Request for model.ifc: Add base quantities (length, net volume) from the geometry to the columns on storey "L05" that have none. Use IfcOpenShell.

First a look at what the model holds.

```python
import ifcopenshell
import ifcopenshell.util.element
import ifcopenshell.util.unit

model = ifcopenshell.open("model.ifc")
print(model.schema)
for unit_type in ("LENGTHUNIT", "AREAUNIT", "VOLUMEUNIT"):
    print(unit_type, ifcopenshell.util.unit.calculate_unit_scale(model, unit_type))
storey = next(s for s in model.by_type("IfcBuildingStorey") if s.Name == "L05")
columns = [e for e in ifcopenshell.util.element.get_decomposition(storey) if e.is_a("IfcColumn")]
for e in sorted(columns, key=lambda e: e.id()):
    print(e.id(), e.is_a(), e.Name, list(ifcopenshell.util.element.get_psets(e, qtos_only=True)), sep=" | ")
```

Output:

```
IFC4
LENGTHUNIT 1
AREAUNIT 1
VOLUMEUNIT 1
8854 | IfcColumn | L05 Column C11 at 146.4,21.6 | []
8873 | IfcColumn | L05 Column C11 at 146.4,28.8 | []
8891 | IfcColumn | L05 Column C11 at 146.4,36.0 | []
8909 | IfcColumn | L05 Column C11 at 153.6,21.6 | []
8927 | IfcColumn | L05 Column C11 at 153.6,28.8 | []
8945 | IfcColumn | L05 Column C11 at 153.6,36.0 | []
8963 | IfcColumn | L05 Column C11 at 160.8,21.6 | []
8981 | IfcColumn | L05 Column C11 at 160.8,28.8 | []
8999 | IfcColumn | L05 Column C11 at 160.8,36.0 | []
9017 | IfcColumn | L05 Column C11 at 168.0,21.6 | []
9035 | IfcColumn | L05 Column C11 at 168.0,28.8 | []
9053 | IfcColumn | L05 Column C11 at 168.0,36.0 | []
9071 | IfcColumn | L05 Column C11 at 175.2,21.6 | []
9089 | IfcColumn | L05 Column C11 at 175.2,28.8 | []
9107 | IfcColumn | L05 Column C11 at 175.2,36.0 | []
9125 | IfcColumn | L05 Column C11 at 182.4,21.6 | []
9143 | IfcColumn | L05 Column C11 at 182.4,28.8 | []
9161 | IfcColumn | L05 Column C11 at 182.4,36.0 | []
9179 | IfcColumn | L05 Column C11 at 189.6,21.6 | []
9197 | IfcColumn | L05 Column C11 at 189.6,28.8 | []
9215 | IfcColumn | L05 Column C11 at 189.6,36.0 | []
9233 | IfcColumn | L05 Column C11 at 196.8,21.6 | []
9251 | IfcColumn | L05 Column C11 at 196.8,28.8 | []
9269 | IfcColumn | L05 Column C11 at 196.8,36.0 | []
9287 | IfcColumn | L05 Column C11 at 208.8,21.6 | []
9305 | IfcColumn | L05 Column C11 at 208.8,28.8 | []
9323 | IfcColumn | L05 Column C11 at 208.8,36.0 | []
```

```python
import ifcopenshell
import ifcopenshell.api.pset
import ifcopenshell.geom
import ifcopenshell.util.element
import ifcopenshell.util.shape
import ifcopenshell.util.unit

model = ifcopenshell.open("model.ifc")
unit_scale = ifcopenshell.util.unit.calculate_unit_scale(model)
volume_scale = ifcopenshell.util.unit.calculate_unit_scale(model, "VOLUMEUNIT")
settings = ifcopenshell.geom.settings()

storey = next(s for s in model.by_type("IfcBuildingStorey") if s.Name == "L05")
columns = [e for e in ifcopenshell.util.element.get_decomposition(storey) if e.is_a("IfcColumn")]

for e in sorted(columns, key=lambda e: e.id()):
    if ifcopenshell.util.element.get_psets(e, qtos_only=True, should_inherit=False):
        continue
    # Geometry comes back in metres, in the element's own axes.
    shape = ifcopenshell.geom.create_shape(settings, e)
    values = {
        "Length": ifcopenshell.util.shape.get_z(shape.geometry) / unit_scale,
        "NetVolume": ifcopenshell.util.shape.get_volume(shape.geometry) / volume_scale,
    }
    qto = ifcopenshell.api.pset.add_qto(model, product=e, name="Qto_ColumnBaseQuantities")
    ifcopenshell.api.pset.edit_qto(model, qto=qto, properties=values)
    print(e.id(), {k: round(v, 3) for k, v in values.items()})

model.write("model_edited.ifc")
```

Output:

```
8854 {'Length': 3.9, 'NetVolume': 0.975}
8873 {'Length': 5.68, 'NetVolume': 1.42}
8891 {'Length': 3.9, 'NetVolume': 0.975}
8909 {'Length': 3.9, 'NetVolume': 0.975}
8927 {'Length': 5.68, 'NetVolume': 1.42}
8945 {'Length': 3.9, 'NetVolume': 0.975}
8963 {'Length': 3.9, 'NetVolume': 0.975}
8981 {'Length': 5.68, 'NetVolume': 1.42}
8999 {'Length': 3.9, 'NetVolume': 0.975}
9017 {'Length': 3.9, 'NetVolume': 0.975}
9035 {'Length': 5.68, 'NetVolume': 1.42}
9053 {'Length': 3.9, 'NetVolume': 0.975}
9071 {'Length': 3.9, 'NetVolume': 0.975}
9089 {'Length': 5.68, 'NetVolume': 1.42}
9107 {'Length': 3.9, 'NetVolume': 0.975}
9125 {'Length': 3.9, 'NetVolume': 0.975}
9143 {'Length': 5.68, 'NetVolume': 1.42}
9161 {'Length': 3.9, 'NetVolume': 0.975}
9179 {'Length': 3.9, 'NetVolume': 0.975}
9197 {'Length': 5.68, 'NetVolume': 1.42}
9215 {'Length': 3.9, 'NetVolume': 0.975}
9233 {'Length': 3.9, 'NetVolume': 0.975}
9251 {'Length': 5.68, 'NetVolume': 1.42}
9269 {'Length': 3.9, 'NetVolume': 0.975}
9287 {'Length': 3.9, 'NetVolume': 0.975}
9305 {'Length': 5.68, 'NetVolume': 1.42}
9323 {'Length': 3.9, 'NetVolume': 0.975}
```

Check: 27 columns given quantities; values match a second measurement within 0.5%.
